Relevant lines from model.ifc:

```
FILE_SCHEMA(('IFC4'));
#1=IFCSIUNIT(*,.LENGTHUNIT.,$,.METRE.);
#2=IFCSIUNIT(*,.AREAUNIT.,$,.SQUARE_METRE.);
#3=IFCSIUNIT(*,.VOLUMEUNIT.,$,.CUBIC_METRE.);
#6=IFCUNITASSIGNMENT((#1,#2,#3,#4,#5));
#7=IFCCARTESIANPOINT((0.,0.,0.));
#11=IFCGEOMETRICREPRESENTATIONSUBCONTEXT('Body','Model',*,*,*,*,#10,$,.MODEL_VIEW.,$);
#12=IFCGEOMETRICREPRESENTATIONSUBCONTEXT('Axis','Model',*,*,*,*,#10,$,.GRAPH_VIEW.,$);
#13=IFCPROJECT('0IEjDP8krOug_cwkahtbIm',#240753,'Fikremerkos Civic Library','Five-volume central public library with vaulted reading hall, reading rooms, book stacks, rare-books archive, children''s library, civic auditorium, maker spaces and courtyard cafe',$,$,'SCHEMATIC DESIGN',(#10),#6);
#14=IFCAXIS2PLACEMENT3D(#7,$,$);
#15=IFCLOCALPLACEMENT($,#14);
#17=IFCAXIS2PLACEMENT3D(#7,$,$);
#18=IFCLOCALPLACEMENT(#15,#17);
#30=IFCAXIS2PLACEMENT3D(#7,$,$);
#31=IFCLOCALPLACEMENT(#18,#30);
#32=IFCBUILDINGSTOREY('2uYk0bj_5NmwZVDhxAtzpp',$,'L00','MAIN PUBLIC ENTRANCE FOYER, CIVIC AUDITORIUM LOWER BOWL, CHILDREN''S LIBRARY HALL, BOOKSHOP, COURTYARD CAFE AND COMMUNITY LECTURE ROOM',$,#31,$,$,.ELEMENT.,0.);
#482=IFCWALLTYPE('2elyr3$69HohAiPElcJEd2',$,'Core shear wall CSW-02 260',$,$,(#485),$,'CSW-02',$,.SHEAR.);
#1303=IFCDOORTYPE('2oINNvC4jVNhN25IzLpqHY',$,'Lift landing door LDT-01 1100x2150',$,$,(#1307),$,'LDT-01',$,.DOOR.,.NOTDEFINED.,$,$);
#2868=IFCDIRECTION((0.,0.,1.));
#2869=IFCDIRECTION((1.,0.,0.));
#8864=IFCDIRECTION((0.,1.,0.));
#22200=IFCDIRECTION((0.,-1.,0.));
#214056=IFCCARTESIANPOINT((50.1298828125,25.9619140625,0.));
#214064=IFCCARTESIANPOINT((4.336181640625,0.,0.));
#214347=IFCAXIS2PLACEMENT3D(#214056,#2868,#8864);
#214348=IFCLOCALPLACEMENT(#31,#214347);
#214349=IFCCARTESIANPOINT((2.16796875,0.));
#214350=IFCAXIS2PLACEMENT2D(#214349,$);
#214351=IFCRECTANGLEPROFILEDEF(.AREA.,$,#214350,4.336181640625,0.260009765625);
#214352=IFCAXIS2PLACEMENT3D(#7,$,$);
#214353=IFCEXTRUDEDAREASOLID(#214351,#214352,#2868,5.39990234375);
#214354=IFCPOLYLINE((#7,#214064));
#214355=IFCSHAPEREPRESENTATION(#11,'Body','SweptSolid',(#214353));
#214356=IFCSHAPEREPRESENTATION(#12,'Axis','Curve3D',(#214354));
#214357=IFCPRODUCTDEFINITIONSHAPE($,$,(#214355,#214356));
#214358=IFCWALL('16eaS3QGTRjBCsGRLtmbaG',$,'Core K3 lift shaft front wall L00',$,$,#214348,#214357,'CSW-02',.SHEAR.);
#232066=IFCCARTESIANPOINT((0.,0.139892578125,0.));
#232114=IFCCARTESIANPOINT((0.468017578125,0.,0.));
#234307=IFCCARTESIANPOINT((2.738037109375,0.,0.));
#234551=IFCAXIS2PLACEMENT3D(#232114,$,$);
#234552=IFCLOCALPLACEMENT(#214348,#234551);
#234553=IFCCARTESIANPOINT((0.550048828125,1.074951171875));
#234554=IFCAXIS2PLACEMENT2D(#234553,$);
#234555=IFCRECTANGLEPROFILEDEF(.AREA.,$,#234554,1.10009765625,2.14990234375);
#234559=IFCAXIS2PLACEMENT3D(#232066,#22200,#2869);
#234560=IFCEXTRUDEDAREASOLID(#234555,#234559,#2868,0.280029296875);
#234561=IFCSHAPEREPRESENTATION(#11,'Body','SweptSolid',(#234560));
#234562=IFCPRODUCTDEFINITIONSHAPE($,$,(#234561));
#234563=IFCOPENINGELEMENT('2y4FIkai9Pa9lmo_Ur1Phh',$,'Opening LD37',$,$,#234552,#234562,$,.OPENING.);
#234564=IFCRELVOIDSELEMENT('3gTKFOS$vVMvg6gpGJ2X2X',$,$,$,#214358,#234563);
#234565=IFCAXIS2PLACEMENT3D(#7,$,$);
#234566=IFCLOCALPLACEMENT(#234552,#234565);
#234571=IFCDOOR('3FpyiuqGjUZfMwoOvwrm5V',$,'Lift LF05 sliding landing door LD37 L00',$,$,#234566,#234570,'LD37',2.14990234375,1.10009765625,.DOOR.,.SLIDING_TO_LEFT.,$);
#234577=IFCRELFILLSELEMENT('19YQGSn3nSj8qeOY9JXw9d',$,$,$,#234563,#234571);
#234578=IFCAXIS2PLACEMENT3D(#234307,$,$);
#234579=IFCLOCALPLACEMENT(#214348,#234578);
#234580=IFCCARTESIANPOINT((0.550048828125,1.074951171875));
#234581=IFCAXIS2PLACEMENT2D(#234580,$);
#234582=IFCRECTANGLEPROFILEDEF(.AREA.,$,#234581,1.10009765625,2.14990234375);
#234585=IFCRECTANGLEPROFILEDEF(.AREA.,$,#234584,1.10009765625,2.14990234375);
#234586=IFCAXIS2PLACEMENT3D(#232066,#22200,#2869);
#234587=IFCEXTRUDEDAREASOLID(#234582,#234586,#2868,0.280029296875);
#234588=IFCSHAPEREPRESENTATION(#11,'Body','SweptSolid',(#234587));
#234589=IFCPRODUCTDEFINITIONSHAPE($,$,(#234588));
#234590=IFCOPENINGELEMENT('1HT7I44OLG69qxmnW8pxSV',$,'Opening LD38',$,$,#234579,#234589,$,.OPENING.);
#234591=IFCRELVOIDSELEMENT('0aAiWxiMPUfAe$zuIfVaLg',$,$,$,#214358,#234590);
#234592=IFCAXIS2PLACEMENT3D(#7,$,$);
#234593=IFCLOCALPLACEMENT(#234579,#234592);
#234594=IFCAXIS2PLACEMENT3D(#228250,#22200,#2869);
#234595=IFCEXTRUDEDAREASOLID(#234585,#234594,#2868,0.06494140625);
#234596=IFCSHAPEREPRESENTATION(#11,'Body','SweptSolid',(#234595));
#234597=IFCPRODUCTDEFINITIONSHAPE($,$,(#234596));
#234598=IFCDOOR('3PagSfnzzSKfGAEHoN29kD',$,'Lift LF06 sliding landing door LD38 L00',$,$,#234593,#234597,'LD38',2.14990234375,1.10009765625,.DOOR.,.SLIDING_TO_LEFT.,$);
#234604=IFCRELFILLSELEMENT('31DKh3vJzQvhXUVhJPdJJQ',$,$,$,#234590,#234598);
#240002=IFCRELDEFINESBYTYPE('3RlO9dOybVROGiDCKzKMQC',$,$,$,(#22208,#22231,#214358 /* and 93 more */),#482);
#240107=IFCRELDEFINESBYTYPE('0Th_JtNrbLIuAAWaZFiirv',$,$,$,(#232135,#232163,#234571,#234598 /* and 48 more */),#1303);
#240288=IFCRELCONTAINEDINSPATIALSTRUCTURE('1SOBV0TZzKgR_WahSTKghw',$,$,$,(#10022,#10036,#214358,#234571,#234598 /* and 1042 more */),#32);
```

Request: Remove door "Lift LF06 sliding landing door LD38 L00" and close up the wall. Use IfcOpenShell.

```python
import ifcopenshell
import ifcopenshell.api.feature
import ifcopenshell.api.root
import ifcopenshell.geom
import ifcopenshell.util.shape

model = ifcopenshell.open("model.ifc")
settings = ifcopenshell.geom.settings()


def volume(element):
    """Net volume in cubic metres, openings subtracted."""
    shape = ifcopenshell.geom.create_shape(settings, element)
    return ifcopenshell.util.shape.get_volume(shape.geometry)


door = model.by_guid("3PagSfnzzSKfGAEHoN29kD")
opening = door.FillsVoids[0].RelatingOpeningElement
wall = opening.VoidsElements[0].RelatingBuildingElement
before = volume(wall)

ifcopenshell.api.root.remove_product(model, product=door)
ifcopenshell.api.feature.remove_feature(model, feature=opening)

after = volume(wall)

print(f"wall volume {before:.3f} -> {after:.3f} m3")

model.write("model_rev.ifc")
```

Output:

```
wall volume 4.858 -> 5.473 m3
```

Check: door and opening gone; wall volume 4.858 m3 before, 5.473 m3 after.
